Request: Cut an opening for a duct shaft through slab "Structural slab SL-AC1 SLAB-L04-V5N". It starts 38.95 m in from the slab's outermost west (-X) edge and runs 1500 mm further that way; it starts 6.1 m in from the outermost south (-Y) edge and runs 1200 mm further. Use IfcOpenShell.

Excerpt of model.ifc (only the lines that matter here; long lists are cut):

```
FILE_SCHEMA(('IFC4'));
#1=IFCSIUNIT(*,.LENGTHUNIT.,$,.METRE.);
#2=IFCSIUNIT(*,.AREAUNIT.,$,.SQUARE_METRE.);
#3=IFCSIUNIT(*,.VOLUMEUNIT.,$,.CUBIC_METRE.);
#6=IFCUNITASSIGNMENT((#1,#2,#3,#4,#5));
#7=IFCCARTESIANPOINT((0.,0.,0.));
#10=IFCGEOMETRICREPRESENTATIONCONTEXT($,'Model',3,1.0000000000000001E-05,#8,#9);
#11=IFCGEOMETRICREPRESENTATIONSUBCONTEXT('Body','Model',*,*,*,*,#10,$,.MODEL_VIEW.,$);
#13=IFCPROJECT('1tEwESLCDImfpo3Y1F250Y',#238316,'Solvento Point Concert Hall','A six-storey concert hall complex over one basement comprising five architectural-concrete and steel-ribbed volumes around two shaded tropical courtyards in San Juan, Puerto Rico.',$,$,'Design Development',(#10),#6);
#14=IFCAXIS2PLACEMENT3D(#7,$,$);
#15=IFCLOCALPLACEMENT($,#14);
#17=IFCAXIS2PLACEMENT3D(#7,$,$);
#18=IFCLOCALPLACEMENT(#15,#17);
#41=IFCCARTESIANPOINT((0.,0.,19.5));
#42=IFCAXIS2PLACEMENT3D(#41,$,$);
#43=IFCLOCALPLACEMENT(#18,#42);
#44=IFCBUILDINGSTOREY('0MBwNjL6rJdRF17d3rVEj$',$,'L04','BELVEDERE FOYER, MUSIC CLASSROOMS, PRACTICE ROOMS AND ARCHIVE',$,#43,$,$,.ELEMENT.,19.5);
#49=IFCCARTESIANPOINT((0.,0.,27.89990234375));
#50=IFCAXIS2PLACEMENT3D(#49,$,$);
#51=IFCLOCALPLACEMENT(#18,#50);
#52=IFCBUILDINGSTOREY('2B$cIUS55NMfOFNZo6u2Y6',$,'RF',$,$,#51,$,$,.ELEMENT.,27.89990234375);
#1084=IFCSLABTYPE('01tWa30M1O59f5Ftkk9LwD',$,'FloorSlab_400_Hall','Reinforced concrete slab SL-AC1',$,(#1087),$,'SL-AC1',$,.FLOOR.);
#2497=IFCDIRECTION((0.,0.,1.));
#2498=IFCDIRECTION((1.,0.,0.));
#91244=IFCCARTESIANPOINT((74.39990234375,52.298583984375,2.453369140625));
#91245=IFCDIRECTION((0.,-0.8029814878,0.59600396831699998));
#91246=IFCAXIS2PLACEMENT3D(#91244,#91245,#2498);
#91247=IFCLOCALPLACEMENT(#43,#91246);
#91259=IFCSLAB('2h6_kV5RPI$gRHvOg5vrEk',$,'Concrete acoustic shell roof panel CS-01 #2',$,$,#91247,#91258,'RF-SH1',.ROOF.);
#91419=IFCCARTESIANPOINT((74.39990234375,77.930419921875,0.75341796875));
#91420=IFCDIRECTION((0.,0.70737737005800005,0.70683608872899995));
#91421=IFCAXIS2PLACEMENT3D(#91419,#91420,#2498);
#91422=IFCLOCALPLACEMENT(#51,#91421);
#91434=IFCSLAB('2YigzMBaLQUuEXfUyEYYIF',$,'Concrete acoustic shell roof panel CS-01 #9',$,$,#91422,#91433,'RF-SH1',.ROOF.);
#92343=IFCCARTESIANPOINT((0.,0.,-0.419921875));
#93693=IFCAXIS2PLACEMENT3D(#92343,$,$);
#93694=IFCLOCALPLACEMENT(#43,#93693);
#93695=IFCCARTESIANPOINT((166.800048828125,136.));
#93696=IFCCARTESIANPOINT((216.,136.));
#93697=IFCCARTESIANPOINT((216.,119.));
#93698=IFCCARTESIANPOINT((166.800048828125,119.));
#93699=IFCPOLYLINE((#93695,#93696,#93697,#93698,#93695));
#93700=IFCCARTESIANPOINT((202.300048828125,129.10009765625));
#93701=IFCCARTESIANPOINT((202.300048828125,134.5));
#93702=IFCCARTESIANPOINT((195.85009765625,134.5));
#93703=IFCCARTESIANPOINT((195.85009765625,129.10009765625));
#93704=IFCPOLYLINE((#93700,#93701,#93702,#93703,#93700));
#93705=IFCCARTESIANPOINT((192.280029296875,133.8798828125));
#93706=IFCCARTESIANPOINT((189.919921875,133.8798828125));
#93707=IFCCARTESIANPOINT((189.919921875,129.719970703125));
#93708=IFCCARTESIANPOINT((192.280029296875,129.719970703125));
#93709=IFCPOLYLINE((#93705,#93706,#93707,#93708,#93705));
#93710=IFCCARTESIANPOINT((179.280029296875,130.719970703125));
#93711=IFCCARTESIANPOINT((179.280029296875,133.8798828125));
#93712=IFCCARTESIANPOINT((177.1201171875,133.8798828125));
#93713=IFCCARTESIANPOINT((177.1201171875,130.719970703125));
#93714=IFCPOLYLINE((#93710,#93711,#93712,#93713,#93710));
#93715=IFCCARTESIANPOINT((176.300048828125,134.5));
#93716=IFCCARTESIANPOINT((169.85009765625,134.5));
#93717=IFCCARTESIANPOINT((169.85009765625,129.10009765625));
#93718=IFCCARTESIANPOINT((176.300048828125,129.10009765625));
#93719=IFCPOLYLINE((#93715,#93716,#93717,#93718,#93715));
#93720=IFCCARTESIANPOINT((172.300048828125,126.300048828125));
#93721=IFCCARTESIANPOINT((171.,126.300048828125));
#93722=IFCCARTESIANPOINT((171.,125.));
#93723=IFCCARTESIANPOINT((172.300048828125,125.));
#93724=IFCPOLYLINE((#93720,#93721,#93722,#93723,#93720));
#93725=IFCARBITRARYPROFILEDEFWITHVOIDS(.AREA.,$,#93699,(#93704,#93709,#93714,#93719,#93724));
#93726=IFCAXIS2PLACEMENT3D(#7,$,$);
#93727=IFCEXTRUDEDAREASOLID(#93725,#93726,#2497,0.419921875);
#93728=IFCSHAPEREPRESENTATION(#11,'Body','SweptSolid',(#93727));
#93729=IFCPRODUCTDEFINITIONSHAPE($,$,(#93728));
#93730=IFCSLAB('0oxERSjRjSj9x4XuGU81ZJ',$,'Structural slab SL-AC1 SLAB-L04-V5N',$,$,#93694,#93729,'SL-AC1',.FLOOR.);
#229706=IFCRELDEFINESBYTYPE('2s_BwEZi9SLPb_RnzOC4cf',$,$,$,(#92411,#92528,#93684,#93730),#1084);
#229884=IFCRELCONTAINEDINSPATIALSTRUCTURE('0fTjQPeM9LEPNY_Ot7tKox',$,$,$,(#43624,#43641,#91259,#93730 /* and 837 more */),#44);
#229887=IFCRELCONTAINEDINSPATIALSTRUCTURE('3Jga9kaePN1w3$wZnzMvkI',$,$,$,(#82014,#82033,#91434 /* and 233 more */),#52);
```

```python
import numpy as np
import ifcopenshell
import ifcopenshell.api.feature
import ifcopenshell.api.geometry
import ifcopenshell.api.root
import ifcopenshell.geom
import ifcopenshell.util.placement
import ifcopenshell.util.representation
import ifcopenshell.util.shape
import ifcopenshell.util.unit

model = ifcopenshell.open("model.ifc")
unit_scale = ifcopenshell.util.unit.calculate_unit_scale(model)
settings = ifcopenshell.geom.settings()


def volume(element):
    """Net volume in cubic metres, openings subtracted."""
    shape = ifcopenshell.geom.create_shape(settings, element)
    return ifcopenshell.util.shape.get_volume(shape.geometry)


slab = model.by_guid("0oxERSjRjSj9x4XuGU81ZJ")
before = volume(slab)

# Extent in the slab's own axes, in metres. The edges named are its -X and -Y sides.
slab_shape = ifcopenshell.geom.create_shape(settings, slab)
vertices = ifcopenshell.util.shape.get_vertices(slab_shape.geometry)
x_min, y_min, bottom = vertices.min(axis=0)
top = vertices[:, 2].max()

opening = ifcopenshell.api.root.create_entity(model, ifc_class="IfcOpeningElement", name="Duct shaft opening", predefined_type="OPENING")
context = ifcopenshell.util.representation.get_context(model, "Model", "Body", "MODEL_VIEW")
width, depth = 1.5, 1.2
outline = [(0.0, 0.0), (width, 0.0), (width, depth), (0.0, depth), (0.0, 0.0)]
# Overshoot both faces by 50 mm so the cut is clean.
shape = ifcopenshell.api.geometry.add_slab_representation(
    model, context=context, depth=top - bottom + 0.1, polyline=outline
)
ifcopenshell.api.geometry.assign_representation(model, product=opening, representation=shape)

matrix = ifcopenshell.util.placement.get_local_placement(slab.ObjectPlacement)
matrix[:, 3] = matrix @ np.append(np.array([x_min + 38.95, y_min + 6.1, bottom - 0.05]) / unit_scale, 1.0)
ifcopenshell.api.geometry.edit_object_placement(model, product=opening, matrix=matrix, is_si=False)
ifcopenshell.api.feature.add_feature(model, feature=opening, element=slab)

after = volume(slab)

print(f"slab volume {before:.3f} -> {after:.3f} m3")

model.write("model_updated.ifc")
```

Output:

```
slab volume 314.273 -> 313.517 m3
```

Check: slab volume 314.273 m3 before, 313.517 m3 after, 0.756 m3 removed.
